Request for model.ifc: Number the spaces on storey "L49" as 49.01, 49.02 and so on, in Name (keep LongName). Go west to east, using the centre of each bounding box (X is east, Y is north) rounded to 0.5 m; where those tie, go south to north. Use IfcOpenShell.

First a look at what the model holds.

```python
import ifcopenshell
import ifcopenshell.util.element
import ifcopenshell.util.placement

model = ifcopenshell.open("model.ifc")
print(model.schema)
storey = next(s for s in model.by_type("IfcBuildingStorey") if s.Name == "L49")
spaces = [e for e in ifcopenshell.util.element.get_decomposition(storey) if e.is_a("IfcSpace")]
for e in sorted(spaces, key=lambda e: e.id()):
    origin = ifcopenshell.util.placement.get_local_placement(e.ObjectPlacement)[:3, 3]
    print(e.id(), e.Name, e.LongName, origin.round(2) + 0.0, sep=" | ")
```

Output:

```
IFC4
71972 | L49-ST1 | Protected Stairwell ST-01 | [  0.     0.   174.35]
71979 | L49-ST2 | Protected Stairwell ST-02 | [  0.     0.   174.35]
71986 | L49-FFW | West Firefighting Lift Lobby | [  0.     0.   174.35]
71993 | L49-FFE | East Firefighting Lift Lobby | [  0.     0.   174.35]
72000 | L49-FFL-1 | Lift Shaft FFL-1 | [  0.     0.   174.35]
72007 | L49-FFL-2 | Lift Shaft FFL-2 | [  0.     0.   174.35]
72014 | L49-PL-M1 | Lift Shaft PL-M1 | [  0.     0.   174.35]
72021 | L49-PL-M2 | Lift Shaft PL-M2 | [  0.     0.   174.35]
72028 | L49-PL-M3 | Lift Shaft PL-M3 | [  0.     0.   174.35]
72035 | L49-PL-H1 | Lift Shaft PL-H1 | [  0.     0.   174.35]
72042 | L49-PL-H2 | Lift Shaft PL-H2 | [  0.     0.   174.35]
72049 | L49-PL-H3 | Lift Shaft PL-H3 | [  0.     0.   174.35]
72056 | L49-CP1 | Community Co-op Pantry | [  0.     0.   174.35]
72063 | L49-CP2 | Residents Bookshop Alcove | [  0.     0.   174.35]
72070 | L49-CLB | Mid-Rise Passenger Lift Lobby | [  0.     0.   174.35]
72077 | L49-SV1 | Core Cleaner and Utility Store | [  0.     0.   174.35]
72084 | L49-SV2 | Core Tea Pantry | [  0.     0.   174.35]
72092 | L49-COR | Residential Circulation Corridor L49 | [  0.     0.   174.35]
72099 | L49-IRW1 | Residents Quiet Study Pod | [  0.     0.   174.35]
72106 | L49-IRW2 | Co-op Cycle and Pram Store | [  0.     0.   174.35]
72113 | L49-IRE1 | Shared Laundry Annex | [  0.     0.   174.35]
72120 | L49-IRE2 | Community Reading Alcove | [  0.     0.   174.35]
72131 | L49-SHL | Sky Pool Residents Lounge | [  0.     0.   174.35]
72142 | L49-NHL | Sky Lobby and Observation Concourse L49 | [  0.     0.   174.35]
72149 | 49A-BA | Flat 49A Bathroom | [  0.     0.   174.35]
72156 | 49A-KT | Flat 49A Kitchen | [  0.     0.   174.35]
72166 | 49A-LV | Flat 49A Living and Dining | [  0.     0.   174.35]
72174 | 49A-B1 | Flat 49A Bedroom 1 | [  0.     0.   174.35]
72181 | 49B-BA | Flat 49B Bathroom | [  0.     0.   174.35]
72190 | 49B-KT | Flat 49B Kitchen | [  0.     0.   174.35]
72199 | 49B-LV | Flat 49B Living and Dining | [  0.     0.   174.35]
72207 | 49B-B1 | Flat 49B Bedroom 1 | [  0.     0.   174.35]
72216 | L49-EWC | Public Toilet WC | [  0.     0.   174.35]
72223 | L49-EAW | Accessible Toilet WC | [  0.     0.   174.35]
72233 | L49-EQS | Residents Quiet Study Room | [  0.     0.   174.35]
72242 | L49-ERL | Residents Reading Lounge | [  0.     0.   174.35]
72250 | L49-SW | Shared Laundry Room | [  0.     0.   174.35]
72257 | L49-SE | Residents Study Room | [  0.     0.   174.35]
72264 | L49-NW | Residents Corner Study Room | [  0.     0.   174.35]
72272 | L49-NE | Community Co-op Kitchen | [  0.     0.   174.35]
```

```python
import ifcopenshell
import ifcopenshell.geom
import ifcopenshell.util.element
import ifcopenshell.util.shape

model = ifcopenshell.open("model.ifc")
settings = ifcopenshell.geom.settings()
settings.set("use-world-coords", True)


def centre(element):
    shape = ifcopenshell.geom.create_shape(settings, element)
    return ifcopenshell.util.shape.get_bbox_centroid(shape.geometry)


storey = next(s for s in model.by_type("IfcBuildingStorey") if s.Name == "L49")
spaces = [e for e in ifcopenshell.util.element.get_decomposition(storey) if e.is_a("IfcSpace")]

# Insertion points can sit at a corner or the storey origin, so sort by the geometry (in metres).
centres = {e: centre(e) for e in spaces}
spaces.sort(key=lambda e: (round(centres[e][0] / 0.5), centres[e][1]))

for i, e in enumerate(spaces, start=1):
    number = f"49.{i:02d}"
    e.Name = number
    print(e.id(), number)

model.write("model_rev.ifc")
```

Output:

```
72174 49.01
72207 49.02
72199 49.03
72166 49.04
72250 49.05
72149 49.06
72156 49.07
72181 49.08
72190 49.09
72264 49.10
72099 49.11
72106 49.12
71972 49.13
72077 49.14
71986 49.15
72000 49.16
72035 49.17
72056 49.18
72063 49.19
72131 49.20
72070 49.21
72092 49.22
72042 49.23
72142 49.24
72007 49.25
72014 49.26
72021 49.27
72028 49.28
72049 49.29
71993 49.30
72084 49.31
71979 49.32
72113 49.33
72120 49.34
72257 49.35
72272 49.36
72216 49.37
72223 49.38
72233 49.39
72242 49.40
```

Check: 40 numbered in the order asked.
